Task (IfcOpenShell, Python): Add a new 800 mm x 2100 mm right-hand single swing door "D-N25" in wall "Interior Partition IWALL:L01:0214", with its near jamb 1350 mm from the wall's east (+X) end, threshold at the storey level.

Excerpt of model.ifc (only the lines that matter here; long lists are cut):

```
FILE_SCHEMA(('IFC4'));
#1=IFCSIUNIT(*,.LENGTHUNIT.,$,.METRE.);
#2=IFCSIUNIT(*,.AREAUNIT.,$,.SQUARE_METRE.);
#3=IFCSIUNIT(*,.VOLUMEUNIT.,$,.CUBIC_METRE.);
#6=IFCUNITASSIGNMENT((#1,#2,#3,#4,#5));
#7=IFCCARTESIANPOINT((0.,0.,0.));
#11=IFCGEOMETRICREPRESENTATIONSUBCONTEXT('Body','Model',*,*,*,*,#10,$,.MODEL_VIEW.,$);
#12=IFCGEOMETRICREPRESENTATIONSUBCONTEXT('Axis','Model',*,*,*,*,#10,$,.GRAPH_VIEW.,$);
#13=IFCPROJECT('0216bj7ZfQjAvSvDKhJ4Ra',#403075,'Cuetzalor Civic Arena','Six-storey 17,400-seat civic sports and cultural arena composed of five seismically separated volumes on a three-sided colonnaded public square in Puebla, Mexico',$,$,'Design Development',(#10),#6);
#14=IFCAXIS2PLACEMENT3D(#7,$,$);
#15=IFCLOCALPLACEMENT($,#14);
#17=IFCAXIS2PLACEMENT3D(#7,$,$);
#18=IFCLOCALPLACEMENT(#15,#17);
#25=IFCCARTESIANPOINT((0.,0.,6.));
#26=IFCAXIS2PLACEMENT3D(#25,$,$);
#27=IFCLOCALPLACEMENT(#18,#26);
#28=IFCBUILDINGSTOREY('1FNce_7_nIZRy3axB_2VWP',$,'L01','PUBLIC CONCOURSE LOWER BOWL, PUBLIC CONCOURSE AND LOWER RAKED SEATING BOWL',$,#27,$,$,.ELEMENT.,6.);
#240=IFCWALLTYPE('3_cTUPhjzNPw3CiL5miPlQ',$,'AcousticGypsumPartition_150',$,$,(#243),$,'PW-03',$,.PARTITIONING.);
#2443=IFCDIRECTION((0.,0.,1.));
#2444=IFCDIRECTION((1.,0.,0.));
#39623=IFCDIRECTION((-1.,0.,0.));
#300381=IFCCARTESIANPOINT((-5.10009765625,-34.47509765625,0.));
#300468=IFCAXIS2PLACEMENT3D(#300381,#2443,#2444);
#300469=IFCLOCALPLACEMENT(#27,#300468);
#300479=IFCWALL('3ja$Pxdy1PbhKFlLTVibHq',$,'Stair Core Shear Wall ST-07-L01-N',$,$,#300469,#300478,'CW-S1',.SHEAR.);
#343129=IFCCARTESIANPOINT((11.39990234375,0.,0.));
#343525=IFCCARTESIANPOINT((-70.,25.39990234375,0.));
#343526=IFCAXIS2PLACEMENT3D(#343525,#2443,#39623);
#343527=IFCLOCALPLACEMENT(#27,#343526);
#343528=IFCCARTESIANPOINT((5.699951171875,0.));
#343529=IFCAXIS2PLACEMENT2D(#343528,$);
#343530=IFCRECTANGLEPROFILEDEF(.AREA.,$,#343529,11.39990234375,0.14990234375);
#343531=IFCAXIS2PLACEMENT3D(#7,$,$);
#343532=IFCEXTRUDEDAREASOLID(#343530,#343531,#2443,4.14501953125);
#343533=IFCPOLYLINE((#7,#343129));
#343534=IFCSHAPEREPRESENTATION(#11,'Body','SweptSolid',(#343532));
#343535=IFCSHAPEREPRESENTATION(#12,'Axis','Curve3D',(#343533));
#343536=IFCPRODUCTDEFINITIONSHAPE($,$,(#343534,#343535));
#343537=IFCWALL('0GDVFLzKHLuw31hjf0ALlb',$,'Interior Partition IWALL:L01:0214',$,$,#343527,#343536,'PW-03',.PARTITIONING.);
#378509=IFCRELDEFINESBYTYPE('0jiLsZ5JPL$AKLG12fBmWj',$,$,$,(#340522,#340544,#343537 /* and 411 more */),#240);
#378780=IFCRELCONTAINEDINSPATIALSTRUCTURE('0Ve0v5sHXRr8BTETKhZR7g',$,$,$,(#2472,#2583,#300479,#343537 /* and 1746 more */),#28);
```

```python
import numpy as np
import ifcopenshell
import ifcopenshell.api.feature
import ifcopenshell.api.geometry
import ifcopenshell.api.root
import ifcopenshell.api.spatial
import ifcopenshell.geom
import ifcopenshell.util.element
import ifcopenshell.util.placement
import ifcopenshell.util.representation
import ifcopenshell.util.shape
import ifcopenshell.util.unit

model = ifcopenshell.open("model.ifc")
unit_scale = ifcopenshell.util.unit.calculate_unit_scale(model)
settings = ifcopenshell.geom.settings()


def volume(element):
    """Net volume in cubic metres, openings subtracted."""
    shape = ifcopenshell.geom.create_shape(settings, element)
    return ifcopenshell.util.shape.get_volume(shape.geometry)


wall = model.by_guid("0GDVFLzKHLuw31hjf0ALlb")
storey = ifcopenshell.util.element.get_container(wall, ifc_class="IfcBuildingStorey")
context = ifcopenshell.util.representation.get_context(model, "Model", "Body", "MODEL_VIEW")
before = volume(wall)

width, height, from_end, sill = 0.8, 2.1, 1.35, 0.0  # metres

# The wall runs along its own X axis, and the end named is its -X end.
wall_shape = ifcopenshell.geom.create_shape(settings, wall)
x, y, z = ifcopenshell.util.shape.get_vertices(wall_shape.geometry).T
start = x.min() + from_end
face, thickness = float(y.min()), float(y.max() - y.min())
wall_matrix = ifcopenshell.util.placement.get_local_placement(wall.ObjectPlacement)
level = ifcopenshell.util.placement.get_local_placement(storey.ObjectPlacement)[2, 3]


def in_wall(x, y):
    """Placement at x, y metres in the wall's axes, at sill height."""
    matrix = wall_matrix.copy()
    matrix[:, 3] = wall_matrix @ np.array([x / unit_scale, y / unit_scale, 0.0, 1.0])
    matrix[2, 3] = level + sill / unit_scale
    return matrix


# Opening: a box that overshoots both wall faces by 50 mm.
opening = ifcopenshell.api.root.create_entity(model, ifc_class="IfcOpeningElement", predefined_type="OPENING")
box = ifcopenshell.api.geometry.add_wall_representation(
    model, context=context, length=width, height=height, thickness=thickness + 0.1
)
ifcopenshell.api.geometry.assign_representation(model, product=opening, representation=box)
ifcopenshell.api.geometry.edit_object_placement(model, product=opening, matrix=in_wall(start, face - 0.05), is_si=False)
ifcopenshell.api.feature.add_feature(model, feature=opening, element=wall)

door = ifcopenshell.api.root.create_entity(model, ifc_class="IfcDoor", name="D-N25", predefined_type="DOOR")
door.OverallWidth, door.OverallHeight = width / unit_scale, height / unit_scale
door.OperationType = "SINGLE_SWING_RIGHT"
body = ifcopenshell.api.geometry.add_door_representation(
    model,
    context=context,
    overall_width=door.OverallWidth,
    overall_height=door.OverallHeight,
    operation_type="SINGLE_SWING_RIGHT",
    lining_properties={"LiningDepth": thickness / unit_scale, "ThresholdDepth": thickness / unit_scale},
)
ifcopenshell.api.geometry.assign_representation(model, product=door, representation=body)
ifcopenshell.api.spatial.assign_container(model, products=[door], relating_structure=storey)
ifcopenshell.api.feature.add_filling(model, opening=opening, element=door)

# The lining spans the wall, so the door starts at the wall face.
ifcopenshell.api.geometry.edit_object_placement(model, product=door, matrix=in_wall(start, face), is_si=False)

after = volume(wall)

print(f"wall volume {before:.3f} -> {after:.3f} m3")

model.write("model_rev.ifc")
```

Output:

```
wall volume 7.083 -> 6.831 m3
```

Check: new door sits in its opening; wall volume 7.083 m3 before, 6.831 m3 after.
